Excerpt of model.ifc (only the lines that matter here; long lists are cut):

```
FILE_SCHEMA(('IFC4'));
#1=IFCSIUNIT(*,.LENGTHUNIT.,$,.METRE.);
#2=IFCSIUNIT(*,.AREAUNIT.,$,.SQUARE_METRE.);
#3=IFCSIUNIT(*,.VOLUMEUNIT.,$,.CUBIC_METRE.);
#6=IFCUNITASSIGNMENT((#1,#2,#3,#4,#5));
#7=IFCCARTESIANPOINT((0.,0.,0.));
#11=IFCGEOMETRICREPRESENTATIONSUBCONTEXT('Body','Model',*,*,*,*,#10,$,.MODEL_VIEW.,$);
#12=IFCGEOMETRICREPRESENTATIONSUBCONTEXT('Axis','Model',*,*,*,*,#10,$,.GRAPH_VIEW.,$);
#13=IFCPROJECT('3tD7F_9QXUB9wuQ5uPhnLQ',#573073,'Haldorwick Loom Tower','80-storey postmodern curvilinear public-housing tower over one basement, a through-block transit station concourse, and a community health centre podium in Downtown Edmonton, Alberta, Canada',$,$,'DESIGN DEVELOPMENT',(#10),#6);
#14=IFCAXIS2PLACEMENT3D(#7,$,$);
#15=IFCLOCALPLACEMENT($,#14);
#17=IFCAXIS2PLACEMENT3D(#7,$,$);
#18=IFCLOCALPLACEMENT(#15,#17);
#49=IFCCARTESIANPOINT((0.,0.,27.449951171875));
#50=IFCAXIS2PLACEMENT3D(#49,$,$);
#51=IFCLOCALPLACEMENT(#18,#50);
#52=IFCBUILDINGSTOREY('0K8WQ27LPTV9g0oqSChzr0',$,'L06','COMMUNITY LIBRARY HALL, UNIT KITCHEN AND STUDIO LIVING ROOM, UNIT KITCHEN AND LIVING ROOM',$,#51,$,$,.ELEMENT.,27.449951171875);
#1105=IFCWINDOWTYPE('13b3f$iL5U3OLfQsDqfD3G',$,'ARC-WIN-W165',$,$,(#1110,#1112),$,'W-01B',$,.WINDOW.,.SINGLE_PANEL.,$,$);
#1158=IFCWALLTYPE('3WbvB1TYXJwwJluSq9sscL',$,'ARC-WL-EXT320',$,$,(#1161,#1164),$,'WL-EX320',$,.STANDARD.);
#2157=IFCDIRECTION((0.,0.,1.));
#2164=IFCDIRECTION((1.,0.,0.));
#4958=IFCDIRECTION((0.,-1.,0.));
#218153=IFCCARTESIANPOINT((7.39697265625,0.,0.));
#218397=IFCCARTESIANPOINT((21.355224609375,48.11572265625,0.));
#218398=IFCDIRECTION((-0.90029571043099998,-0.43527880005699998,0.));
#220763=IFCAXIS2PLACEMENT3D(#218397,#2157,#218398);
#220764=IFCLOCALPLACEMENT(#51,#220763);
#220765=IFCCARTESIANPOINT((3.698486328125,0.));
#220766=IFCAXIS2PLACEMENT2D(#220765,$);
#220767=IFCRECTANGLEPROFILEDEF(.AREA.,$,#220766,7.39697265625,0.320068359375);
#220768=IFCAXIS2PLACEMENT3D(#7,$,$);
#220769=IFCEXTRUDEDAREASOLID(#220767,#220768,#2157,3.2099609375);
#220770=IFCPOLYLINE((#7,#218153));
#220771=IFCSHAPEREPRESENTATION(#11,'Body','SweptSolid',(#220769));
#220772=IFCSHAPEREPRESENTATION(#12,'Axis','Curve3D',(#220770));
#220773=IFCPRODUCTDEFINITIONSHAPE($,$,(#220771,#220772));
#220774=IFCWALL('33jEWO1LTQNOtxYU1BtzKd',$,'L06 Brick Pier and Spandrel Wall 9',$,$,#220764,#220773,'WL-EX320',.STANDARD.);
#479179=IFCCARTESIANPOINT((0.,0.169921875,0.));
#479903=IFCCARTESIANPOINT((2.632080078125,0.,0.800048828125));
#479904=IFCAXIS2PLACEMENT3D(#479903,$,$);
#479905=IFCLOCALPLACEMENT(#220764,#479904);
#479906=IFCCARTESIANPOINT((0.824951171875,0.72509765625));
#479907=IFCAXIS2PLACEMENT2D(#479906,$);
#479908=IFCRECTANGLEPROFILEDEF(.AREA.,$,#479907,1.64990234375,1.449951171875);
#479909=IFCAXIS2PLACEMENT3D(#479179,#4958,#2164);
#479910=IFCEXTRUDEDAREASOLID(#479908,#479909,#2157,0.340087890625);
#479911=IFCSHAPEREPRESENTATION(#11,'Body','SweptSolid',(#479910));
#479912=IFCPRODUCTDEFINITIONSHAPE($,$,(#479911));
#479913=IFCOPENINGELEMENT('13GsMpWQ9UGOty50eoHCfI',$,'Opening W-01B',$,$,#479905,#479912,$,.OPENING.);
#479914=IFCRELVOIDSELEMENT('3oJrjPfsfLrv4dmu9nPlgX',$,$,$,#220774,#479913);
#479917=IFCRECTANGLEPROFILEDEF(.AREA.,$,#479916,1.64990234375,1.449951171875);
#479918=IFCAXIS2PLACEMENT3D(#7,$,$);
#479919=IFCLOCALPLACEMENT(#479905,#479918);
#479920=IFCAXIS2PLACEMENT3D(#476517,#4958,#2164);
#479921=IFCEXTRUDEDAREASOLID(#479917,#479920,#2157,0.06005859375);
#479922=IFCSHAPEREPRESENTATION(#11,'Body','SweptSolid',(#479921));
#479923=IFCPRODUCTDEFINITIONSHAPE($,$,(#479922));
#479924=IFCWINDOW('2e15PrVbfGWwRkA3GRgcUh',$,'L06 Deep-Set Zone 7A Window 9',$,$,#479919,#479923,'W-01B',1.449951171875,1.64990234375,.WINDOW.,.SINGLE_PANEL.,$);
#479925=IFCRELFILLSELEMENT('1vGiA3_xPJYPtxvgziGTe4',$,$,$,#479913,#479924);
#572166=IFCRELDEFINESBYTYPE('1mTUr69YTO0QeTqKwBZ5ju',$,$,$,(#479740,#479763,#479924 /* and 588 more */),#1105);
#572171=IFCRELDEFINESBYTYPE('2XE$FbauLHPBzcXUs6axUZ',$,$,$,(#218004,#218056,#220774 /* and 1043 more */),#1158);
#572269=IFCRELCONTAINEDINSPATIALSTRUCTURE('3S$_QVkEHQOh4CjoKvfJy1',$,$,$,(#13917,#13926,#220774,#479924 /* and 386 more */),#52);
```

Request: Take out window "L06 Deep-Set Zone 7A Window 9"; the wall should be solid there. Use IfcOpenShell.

```python
import ifcopenshell
import ifcopenshell.api.feature
import ifcopenshell.api.root
import ifcopenshell.geom
import ifcopenshell.util.shape

model = ifcopenshell.open("model.ifc")
settings = ifcopenshell.geom.settings()


def volume(element):
    """Net volume in cubic metres, openings subtracted."""
    shape = ifcopenshell.geom.create_shape(settings, element)
    return ifcopenshell.util.shape.get_volume(shape.geometry)


window = model.by_guid("2e15PrVbfGWwRkA3GRgcUh")
opening = window.FillsVoids[0].RelatingOpeningElement
wall = opening.VoidsElements[0].RelatingBuildingElement
before = volume(wall)

ifcopenshell.api.root.remove_product(model, product=window)
ifcopenshell.api.feature.remove_feature(model, feature=opening)

after = volume(wall)

print(f"wall volume {before:.3f} -> {after:.3f} m3")

model.write("model_v2.ifc")
```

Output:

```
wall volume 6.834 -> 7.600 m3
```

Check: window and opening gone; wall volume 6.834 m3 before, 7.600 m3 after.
